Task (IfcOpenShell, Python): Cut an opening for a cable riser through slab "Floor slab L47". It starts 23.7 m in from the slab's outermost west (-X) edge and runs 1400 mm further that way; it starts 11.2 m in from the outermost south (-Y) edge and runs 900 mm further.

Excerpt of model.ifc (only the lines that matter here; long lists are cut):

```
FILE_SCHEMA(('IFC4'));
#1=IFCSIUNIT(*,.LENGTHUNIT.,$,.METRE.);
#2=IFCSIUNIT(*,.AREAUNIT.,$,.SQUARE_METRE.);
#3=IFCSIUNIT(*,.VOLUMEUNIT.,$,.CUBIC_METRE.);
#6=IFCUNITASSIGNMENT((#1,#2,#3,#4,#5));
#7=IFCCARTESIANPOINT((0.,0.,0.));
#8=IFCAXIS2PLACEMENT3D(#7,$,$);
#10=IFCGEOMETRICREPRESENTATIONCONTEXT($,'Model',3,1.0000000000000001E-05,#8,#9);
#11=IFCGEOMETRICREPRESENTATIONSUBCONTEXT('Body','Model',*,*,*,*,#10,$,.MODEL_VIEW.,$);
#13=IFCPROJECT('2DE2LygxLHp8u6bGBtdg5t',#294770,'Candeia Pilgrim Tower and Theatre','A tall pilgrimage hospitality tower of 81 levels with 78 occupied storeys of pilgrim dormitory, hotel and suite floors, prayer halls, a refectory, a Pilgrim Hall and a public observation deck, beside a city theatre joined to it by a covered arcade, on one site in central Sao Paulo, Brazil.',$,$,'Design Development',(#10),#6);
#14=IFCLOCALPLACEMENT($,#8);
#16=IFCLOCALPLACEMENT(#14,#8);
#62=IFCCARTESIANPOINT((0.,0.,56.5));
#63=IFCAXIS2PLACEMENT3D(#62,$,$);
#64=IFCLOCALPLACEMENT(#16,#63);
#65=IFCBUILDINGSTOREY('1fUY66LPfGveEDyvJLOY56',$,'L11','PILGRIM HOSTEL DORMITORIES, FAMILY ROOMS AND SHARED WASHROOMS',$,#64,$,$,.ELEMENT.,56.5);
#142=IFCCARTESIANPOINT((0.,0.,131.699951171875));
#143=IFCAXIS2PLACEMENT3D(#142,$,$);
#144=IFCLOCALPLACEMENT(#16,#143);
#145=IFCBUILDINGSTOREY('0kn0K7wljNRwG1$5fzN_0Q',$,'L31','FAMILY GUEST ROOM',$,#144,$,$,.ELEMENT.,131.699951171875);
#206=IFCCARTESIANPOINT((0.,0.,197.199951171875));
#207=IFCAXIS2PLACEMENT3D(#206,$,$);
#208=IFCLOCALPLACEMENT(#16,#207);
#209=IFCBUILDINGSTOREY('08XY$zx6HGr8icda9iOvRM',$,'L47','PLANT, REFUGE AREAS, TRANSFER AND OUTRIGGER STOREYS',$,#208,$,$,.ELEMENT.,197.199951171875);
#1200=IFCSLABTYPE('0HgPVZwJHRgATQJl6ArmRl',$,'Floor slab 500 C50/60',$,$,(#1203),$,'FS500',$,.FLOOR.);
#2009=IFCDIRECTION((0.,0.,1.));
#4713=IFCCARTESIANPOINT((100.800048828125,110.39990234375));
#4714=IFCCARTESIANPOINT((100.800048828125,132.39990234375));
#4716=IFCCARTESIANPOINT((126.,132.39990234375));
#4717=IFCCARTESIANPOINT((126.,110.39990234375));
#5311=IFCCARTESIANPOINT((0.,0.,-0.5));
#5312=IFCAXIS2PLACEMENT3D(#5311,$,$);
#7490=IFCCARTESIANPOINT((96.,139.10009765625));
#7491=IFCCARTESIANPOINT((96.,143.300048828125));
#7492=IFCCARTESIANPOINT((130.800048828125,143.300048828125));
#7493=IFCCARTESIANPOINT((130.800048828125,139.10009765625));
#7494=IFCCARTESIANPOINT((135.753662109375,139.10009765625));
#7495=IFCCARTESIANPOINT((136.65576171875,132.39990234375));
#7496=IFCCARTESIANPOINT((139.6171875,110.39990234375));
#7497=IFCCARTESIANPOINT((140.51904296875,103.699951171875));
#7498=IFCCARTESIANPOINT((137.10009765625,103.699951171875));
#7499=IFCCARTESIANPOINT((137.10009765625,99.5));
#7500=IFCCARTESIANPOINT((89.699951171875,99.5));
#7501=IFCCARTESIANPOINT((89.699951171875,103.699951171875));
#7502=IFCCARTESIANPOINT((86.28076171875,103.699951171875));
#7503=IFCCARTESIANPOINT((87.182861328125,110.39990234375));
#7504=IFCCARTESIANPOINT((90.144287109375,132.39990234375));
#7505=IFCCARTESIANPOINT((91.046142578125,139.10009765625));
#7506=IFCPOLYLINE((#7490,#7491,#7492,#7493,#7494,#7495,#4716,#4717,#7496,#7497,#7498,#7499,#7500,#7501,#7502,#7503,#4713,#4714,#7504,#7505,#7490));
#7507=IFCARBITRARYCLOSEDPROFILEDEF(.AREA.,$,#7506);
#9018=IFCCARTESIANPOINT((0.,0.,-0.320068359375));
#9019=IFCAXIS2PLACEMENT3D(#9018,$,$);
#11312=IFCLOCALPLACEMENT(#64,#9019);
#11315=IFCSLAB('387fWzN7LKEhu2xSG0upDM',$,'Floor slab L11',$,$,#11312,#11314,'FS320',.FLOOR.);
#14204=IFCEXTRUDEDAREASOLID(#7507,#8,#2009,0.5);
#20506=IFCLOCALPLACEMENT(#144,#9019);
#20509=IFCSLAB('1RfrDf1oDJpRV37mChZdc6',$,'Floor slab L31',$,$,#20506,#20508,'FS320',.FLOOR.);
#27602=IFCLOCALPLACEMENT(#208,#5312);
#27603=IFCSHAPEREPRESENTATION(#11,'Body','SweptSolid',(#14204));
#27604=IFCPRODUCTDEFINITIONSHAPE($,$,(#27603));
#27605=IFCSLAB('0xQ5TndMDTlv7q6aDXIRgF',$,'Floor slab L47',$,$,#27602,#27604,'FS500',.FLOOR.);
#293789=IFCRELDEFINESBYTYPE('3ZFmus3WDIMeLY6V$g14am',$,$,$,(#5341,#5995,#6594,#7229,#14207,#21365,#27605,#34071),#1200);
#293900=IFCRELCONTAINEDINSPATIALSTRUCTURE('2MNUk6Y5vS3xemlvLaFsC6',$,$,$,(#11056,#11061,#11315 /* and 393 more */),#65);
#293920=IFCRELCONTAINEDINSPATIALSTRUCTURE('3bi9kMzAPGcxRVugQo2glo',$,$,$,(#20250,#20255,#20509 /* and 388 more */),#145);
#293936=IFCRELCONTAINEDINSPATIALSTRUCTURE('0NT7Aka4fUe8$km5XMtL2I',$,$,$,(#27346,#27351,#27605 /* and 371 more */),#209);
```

```python
import numpy as np
import ifcopenshell
import ifcopenshell.api.feature
import ifcopenshell.api.geometry
import ifcopenshell.api.root
import ifcopenshell.geom
import ifcopenshell.util.placement
import ifcopenshell.util.representation
import ifcopenshell.util.shape
import ifcopenshell.util.unit

model = ifcopenshell.open("model.ifc")
unit_scale = ifcopenshell.util.unit.calculate_unit_scale(model)
settings = ifcopenshell.geom.settings()


def volume(element):
    """Net volume in cubic metres, openings subtracted."""
    shape = ifcopenshell.geom.create_shape(settings, element)
    return ifcopenshell.util.shape.get_volume(shape.geometry)


slab = model.by_guid("0xQ5TndMDTlv7q6aDXIRgF")
before = volume(slab)

# Extent in the slab's own axes, in metres. The edges named are its -X and -Y sides.
slab_shape = ifcopenshell.geom.create_shape(settings, slab)
vertices = ifcopenshell.util.shape.get_vertices(slab_shape.geometry)
x_min, y_min, bottom = vertices.min(axis=0)
top = vertices[:, 2].max()

opening = ifcopenshell.api.root.create_entity(model, ifc_class="IfcOpeningElement", name="Cable riser opening", predefined_type="OPENING")
context = ifcopenshell.util.representation.get_context(model, "Model", "Body", "MODEL_VIEW")
width, depth = 1.4, 0.9
outline = [(0.0, 0.0), (width, 0.0), (width, depth), (0.0, depth), (0.0, 0.0)]
# Overshoot both faces by 50 mm so the cut is clean.
shape = ifcopenshell.api.geometry.add_slab_representation(
    model, context=context, depth=top - bottom + 0.1, polyline=outline
)
ifcopenshell.api.geometry.assign_representation(model, product=opening, representation=shape)

matrix = ifcopenshell.util.placement.get_local_placement(slab.ObjectPlacement)
matrix[:, 3] = matrix @ np.append(np.array([x_min + 23.7, y_min + 11.2, bottom - 0.05]) / unit_scale, 1.0)
ifcopenshell.api.geometry.edit_object_placement(model, product=opening, matrix=matrix, is_si=False)
ifcopenshell.api.feature.add_feature(model, feature=opening, element=slab)

after = volume(slab)

print(f"slab volume {before:.3f} -> {after:.3f} m3")

model.write("model_edited.ifc")
```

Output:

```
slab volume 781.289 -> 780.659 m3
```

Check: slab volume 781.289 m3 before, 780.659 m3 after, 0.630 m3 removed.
